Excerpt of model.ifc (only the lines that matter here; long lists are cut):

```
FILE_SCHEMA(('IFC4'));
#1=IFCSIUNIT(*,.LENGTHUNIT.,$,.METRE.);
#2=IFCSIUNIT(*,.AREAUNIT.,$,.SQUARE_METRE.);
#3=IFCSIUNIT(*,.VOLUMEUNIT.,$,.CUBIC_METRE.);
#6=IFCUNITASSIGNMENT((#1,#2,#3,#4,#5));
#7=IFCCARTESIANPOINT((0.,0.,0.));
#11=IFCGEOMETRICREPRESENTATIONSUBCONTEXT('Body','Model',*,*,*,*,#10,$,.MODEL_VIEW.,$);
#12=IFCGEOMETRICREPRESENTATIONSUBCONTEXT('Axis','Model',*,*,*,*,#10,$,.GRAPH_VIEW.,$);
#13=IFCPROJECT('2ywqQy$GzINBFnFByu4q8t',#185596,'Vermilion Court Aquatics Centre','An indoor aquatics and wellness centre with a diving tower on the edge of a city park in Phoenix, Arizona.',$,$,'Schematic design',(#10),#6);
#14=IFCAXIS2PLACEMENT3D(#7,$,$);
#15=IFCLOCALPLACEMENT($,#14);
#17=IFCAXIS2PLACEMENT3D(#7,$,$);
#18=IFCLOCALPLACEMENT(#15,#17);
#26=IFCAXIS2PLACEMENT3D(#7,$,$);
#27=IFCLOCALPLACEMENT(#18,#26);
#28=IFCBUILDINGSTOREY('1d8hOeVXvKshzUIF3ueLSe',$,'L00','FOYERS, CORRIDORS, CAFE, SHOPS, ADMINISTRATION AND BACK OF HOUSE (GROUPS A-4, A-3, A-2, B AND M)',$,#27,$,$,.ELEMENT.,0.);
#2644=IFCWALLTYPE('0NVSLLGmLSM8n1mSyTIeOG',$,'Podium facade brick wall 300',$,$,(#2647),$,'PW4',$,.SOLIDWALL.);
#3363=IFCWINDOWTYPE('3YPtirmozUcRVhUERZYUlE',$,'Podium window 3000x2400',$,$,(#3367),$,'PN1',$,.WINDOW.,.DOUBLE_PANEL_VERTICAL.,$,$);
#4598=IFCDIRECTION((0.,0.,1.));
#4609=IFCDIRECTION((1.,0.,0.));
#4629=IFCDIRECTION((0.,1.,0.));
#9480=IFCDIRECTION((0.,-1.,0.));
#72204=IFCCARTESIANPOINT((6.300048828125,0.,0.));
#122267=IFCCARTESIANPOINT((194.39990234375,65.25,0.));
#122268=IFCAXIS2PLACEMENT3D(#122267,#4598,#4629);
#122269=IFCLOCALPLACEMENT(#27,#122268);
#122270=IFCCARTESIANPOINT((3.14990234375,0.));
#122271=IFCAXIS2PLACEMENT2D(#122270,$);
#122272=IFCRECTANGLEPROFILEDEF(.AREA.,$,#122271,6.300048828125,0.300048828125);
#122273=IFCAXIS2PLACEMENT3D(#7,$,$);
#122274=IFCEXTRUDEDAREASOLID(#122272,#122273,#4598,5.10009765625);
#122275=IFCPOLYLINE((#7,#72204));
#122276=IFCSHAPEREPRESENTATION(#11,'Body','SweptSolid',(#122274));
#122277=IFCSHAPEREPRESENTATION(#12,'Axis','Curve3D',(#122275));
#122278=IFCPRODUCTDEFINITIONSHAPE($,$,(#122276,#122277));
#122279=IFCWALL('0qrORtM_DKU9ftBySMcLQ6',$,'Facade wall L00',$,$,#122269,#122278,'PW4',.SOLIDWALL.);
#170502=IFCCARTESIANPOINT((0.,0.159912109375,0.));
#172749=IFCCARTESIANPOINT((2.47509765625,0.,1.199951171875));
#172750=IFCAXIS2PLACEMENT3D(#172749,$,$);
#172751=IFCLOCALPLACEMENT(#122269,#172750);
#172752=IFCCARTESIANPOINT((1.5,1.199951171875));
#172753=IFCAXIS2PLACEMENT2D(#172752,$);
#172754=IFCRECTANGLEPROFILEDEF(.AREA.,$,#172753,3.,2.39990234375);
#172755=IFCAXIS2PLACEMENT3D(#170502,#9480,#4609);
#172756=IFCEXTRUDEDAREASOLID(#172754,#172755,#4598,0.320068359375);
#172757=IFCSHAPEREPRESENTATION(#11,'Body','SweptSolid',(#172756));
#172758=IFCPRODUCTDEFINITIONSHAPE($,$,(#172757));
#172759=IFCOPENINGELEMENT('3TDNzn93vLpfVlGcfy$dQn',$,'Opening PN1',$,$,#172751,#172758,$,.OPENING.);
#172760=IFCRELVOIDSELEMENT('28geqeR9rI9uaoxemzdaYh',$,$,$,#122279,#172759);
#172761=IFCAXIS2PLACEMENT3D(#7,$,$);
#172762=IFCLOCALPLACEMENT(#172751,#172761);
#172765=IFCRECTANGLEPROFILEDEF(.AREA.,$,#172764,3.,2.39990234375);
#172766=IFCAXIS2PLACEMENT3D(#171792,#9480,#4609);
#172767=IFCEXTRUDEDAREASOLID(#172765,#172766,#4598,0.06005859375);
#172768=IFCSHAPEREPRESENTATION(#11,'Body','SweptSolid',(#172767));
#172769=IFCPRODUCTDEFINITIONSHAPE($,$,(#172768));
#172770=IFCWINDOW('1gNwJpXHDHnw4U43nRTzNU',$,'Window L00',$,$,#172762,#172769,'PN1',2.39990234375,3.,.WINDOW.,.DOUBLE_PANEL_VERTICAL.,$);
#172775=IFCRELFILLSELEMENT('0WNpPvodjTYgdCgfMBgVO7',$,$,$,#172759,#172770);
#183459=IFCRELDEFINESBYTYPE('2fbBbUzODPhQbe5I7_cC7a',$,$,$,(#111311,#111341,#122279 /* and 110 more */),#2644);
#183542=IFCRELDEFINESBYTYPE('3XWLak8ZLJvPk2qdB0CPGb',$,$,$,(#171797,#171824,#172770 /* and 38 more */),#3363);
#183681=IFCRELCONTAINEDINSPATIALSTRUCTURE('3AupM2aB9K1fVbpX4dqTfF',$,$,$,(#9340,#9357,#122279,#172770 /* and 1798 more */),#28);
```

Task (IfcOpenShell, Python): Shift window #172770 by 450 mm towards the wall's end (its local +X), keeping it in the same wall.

```python
import ifcopenshell
import ifcopenshell.api.geometry
import ifcopenshell.util.placement
import ifcopenshell.util.unit

model = ifcopenshell.open("model.ifc")
unit_scale = ifcopenshell.util.unit.calculate_unit_scale(model)

window = model.by_guid("1gNwJpXHDHnw4U43nRTzNU")
opening = window.FillsVoids[0].RelatingOpeningElement
wall = opening.VoidsElements[0].RelatingBuildingElement

wall_matrix = ifcopenshell.util.placement.get_local_placement(wall.ObjectPlacement)
shift = wall_matrix[:3, 0] * 0.45 / unit_scale
before = ifcopenshell.util.placement.get_local_placement(window.ObjectPlacement)[:3, 3].copy()

# The window is placed relative to its opening, so it follows when the opening moves.
matrix = ifcopenshell.util.placement.get_local_placement(opening.ObjectPlacement)
matrix[:3, 3] += shift
ifcopenshell.api.geometry.edit_object_placement(
    model, product=opening, matrix=matrix, is_si=False, should_transform_children=True
)

after = ifcopenshell.util.placement.get_local_placement(window.ObjectPlacement)[:3, 3]
print("window moved by", (after - before).round(3) + 0.0)

model.write("model_rev.ifc")
```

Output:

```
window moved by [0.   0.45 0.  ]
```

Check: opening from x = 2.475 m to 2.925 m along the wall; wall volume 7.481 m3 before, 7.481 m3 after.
